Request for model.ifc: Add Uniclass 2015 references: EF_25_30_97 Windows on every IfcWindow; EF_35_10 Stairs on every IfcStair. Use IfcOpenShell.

First a look at what the model holds.

```python
import ifcopenshell

model = ifcopenshell.open("model.ifc")
print(model.schema)
print("classifications:", [c.Name for c in model.by_type("IfcClassification")])
for ifc_class in ("IfcDoor", "IfcRoof", "IfcStair", "IfcWall", "IfcWindow"):
    print(ifc_class, len(model.by_type(ifc_class)))
```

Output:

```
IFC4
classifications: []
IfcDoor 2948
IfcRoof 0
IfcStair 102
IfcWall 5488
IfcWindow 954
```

```python
import ifcopenshell
import ifcopenshell.api.classification

model = ifcopenshell.open("model.ifc")

system = ifcopenshell.api.classification.add_classification(model, classification="Uniclass 2015")

codes = {
    "IfcWindow": ("EF_25_30_97", "Windows"),
    "IfcStair": ("EF_35_10", "Stairs"),
}
for ifc_class, (code, name) in codes.items():
    products = model.by_type(ifc_class)
    ifcopenshell.api.classification.add_reference(
        model, products=products, classification=system, identification=code, name=name
    )
    print(code, len(products))

model.write("model-out.ifc")
```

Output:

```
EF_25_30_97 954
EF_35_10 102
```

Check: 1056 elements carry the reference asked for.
